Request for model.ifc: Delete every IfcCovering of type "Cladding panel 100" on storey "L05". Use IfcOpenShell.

First a look at what the model holds.

```python
import ifcopenshell
import ifcopenshell.util.element

model = ifcopenshell.open("model.ifc")
print(model.schema)
storey = next(s for s in model.by_type("IfcBuildingStorey") if s.Name == "L05")
coverings = [e for e in ifcopenshell.util.element.get_decomposition(storey) if e.is_a("IfcCovering")]
seen = {}
for e in coverings:
    element_type = ifcopenshell.util.element.get_type(e)
    name = element_type.Name if element_type not in (None, e) else None
    seen[name] = seen.get(name, 0) + 1
for name, count in sorted(seen.items(), key=str):
    print(count, "x", name)
```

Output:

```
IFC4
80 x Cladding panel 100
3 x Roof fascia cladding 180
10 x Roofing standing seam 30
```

```python
import ifcopenshell
import ifcopenshell.api.root
import ifcopenshell.util.element

model = ifcopenshell.open("model.ifc")

storey = next(s for s in model.by_type("IfcBuildingStorey") if s.Name == "L05")
coverings = [e for e in ifcopenshell.util.element.get_decomposition(storey) if e.is_a("IfcCovering")]
targets = [e for e in coverings if (t := ifcopenshell.util.element.get_type(e)) not in (None, e) and t.Name == "Cladding panel 100"]

for e in targets:
    ifcopenshell.api.root.remove_product(model, product=e)
print(len(targets), "removed")

model.write("model_rev.ifc")
```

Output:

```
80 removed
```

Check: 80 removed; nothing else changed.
